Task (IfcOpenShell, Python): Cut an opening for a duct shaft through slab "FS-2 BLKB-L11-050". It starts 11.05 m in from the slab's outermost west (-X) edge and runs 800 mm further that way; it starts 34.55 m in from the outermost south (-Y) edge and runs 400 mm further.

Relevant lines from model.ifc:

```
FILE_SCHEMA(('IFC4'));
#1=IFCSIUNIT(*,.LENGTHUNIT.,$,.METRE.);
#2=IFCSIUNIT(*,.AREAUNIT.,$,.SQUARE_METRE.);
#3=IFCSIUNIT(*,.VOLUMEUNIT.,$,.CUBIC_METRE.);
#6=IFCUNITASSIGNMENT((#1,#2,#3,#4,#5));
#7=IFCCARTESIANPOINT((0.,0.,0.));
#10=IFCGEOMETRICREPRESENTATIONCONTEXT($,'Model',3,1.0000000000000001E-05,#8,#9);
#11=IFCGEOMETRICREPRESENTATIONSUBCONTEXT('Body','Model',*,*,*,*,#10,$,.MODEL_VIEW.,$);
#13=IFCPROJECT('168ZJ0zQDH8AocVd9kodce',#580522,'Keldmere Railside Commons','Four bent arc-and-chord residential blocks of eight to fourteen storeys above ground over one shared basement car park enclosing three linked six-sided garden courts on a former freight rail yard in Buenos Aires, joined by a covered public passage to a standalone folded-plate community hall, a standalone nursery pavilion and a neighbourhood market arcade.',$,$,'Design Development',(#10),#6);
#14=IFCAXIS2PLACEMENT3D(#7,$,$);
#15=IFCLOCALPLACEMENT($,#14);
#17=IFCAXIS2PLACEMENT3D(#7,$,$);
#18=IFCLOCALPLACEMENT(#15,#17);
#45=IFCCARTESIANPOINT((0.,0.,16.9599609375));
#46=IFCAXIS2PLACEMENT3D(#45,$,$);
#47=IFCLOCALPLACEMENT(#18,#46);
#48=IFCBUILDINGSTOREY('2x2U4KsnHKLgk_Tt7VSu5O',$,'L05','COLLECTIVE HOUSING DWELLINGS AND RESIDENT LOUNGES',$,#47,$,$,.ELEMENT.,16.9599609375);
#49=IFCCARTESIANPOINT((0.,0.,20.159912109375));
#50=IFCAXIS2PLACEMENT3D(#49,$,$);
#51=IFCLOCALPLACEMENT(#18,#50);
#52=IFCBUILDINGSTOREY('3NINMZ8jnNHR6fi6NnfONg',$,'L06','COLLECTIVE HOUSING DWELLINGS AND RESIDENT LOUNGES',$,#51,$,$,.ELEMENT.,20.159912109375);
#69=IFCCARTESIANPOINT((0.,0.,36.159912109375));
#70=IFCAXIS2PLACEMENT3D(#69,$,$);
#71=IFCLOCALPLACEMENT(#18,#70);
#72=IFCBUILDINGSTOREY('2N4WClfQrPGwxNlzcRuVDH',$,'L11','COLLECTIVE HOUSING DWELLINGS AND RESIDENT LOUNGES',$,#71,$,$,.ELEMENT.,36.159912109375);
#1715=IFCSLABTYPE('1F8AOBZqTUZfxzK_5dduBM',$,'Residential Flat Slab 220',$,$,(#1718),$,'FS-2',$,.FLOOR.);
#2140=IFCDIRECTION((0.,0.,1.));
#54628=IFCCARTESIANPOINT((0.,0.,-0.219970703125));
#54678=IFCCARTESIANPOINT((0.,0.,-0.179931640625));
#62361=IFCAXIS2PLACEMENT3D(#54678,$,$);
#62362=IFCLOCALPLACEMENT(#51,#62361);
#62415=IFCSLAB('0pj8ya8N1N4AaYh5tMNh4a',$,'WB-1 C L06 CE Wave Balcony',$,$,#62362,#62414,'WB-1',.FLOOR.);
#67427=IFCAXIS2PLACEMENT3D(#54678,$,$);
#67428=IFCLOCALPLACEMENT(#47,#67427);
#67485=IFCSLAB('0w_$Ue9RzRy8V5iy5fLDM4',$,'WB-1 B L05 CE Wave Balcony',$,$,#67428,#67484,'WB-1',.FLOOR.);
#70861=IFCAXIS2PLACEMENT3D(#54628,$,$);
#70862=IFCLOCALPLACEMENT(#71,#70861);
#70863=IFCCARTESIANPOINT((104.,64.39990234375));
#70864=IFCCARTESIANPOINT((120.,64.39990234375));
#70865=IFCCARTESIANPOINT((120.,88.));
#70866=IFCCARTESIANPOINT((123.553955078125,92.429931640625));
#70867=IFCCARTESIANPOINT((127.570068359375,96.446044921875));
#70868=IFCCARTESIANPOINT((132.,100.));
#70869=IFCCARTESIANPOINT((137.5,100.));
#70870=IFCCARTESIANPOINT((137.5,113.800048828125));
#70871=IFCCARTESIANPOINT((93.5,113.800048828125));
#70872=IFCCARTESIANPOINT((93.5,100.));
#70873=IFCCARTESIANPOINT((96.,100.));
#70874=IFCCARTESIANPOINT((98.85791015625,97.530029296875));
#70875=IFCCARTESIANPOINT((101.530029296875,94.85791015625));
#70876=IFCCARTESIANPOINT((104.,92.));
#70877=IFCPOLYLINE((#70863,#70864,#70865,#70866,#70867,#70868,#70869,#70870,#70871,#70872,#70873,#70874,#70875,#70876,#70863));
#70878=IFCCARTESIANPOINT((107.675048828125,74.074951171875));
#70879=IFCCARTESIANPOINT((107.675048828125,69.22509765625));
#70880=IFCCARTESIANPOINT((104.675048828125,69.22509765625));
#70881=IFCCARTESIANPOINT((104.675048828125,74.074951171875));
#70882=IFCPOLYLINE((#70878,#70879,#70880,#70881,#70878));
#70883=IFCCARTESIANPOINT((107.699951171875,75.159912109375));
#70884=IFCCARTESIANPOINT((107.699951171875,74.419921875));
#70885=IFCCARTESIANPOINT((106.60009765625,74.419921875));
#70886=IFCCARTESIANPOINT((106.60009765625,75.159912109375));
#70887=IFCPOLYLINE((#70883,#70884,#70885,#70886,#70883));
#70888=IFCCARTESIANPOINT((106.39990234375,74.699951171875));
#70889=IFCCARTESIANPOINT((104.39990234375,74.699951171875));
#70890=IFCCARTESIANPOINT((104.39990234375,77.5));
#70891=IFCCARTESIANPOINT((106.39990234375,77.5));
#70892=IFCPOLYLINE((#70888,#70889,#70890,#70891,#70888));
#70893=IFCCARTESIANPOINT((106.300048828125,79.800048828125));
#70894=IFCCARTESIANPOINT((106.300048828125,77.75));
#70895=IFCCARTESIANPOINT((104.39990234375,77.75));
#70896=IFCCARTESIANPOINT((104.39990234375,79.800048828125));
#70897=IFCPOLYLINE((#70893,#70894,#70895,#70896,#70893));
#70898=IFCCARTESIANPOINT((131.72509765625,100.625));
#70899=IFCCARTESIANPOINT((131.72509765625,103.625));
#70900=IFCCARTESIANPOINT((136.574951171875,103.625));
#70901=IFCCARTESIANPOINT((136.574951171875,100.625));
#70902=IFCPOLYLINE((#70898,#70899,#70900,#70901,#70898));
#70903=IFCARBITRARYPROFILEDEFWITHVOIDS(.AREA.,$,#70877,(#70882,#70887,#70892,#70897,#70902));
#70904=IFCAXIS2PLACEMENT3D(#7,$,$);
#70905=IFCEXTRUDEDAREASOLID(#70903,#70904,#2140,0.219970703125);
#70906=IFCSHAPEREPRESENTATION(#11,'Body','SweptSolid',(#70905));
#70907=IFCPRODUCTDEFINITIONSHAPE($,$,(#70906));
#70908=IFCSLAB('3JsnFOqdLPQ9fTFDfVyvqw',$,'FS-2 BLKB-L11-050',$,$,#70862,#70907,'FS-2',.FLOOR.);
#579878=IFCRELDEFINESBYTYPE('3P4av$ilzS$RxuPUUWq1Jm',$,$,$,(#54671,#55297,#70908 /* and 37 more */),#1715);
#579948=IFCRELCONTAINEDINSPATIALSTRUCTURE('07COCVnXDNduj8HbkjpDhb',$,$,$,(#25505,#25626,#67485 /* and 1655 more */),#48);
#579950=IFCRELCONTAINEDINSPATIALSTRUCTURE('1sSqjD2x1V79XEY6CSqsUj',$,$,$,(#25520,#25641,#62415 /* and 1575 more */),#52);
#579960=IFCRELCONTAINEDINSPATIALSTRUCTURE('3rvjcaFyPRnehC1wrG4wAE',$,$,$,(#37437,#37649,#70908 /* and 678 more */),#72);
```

```python
import numpy as np
import ifcopenshell
import ifcopenshell.api.feature
import ifcopenshell.api.geometry
import ifcopenshell.api.root
import ifcopenshell.geom
import ifcopenshell.util.placement
import ifcopenshell.util.representation
import ifcopenshell.util.shape
import ifcopenshell.util.unit

model = ifcopenshell.open("model.ifc")
unit_scale = ifcopenshell.util.unit.calculate_unit_scale(model)
settings = ifcopenshell.geom.settings()


def volume(element):
    """Net volume in cubic metres, openings subtracted."""
    shape = ifcopenshell.geom.create_shape(settings, element)
    return ifcopenshell.util.shape.get_volume(shape.geometry)


slab = model.by_guid("3JsnFOqdLPQ9fTFDfVyvqw")
before = volume(slab)

# Extent in the slab's own axes, in metres. The edges named are its -X and -Y sides.
slab_shape = ifcopenshell.geom.create_shape(settings, slab)
vertices = ifcopenshell.util.shape.get_vertices(slab_shape.geometry)
x_min, y_min, bottom = vertices.min(axis=0)
top = vertices[:, 2].max()

opening = ifcopenshell.api.root.create_entity(model, ifc_class="IfcOpeningElement", name="Duct shaft opening", predefined_type="OPENING")
context = ifcopenshell.util.representation.get_context(model, "Model", "Body", "MODEL_VIEW")
width, depth = 0.8, 0.4
outline = [(0.0, 0.0), (width, 0.0), (width, depth), (0.0, depth), (0.0, 0.0)]
# Overshoot both faces by 50 mm so the cut is clean.
shape = ifcopenshell.api.geometry.add_slab_representation(
    model, context=context, depth=top - bottom + 0.1, polyline=outline
)
ifcopenshell.api.geometry.assign_representation(model, product=opening, representation=shape)

matrix = ifcopenshell.util.placement.get_local_placement(slab.ObjectPlacement)
matrix[:, 3] = matrix @ np.append(np.array([x_min + 11.05, y_min + 34.55, bottom - 0.05]) / unit_scale, 1.0)
ifcopenshell.api.geometry.edit_object_placement(model, product=opening, matrix=matrix, is_si=False)
ifcopenshell.api.feature.add_feature(model, feature=opening, element=slab)

after = volume(slab)

print(f"slab volume {before:.3f} -> {after:.3f} m3")

model.write("model_v2.ifc")
```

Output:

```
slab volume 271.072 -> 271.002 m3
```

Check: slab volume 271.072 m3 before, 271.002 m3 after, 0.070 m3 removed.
